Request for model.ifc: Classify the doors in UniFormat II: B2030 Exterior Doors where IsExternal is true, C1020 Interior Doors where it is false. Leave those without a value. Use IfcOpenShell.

First a look at what the model holds.

```python
import ifcopenshell
import ifcopenshell.util.element

model = ifcopenshell.open("model.ifc")
print(model.schema)
print("classifications:", [c.Name for c in model.by_type("IfcClassification")])
values = [ifcopenshell.util.element.get_pset(e, "Pset_DoorCommon", "IsExternal") for e in model.by_type("IfcDoor")]
for value in (True, False, None):
    print("IsExternal", value, values.count(value))
```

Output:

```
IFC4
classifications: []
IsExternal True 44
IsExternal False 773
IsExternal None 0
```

```python
import ifcopenshell
import ifcopenshell.api.classification
import ifcopenshell.util.element

model = ifcopenshell.open("model.ifc")

system = ifcopenshell.api.classification.add_classification(model, classification="UniFormat II")

doors = model.by_type("IfcDoor")
external = {e: ifcopenshell.util.element.get_pset(e, "Pset_DoorCommon", "IsExternal") for e in doors}
for flag, code, name in ((True, "B2030", "Exterior Doors"), (False, "C1020", "Interior Doors")):
    products = [e for e in doors if external[e] is flag]
    ifcopenshell.api.classification.add_reference(
        model, products=products, classification=system, identification=code, name=name
    )
    print(code, len(products))

model.write("model_updated.ifc")
```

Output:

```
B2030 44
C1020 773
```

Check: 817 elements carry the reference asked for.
